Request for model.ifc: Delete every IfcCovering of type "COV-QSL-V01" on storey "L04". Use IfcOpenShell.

First a look at what the model holds.

```python
import ifcopenshell
import ifcopenshell.util.element

model = ifcopenshell.open("model.ifc")
print(model.schema)
storey = next(s for s in model.by_type("IfcBuildingStorey") if s.Name == "L04")
coverings = [e for e in ifcopenshell.util.element.get_decomposition(storey) if e.is_a("IfcCovering")]
seen = {}
for e in coverings:
    element_type = ifcopenshell.util.element.get_type(e)
    name = element_type.Name if element_type not in (None, e) else None
    seen[name] = seen.get(name, 0) + 1
for name, count in sorted(seen.items(), key=str):
    print(count, "x", name)
```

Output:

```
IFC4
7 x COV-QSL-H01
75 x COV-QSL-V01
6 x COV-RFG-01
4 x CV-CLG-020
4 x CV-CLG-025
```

```python
import ifcopenshell
import ifcopenshell.api.root
import ifcopenshell.util.element

model = ifcopenshell.open("model.ifc")

storey = next(s for s in model.by_type("IfcBuildingStorey") if s.Name == "L04")
coverings = [e for e in ifcopenshell.util.element.get_decomposition(storey) if e.is_a("IfcCovering")]
targets = [e for e in coverings if (t := ifcopenshell.util.element.get_type(e)) not in (None, e) and t.Name == "COV-QSL-V01"]

for e in targets:
    ifcopenshell.api.root.remove_product(model, product=e)
print(len(targets), "removed")

model.write("model_edited.ifc")
```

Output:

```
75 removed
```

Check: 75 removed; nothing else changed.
